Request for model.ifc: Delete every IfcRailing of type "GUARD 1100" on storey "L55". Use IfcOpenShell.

First a look at what the model holds.

```python
import ifcopenshell
import ifcopenshell.util.element

model = ifcopenshell.open("model.ifc")
print(model.schema)
storey = next(s for s in model.by_type("IfcBuildingStorey") if s.Name == "L55")
railings = [e for e in ifcopenshell.util.element.get_decomposition(storey) if e.is_a("IfcRailing")]
seen = {}
for e in railings:
    element_type = ifcopenshell.util.element.get_type(e)
    name = element_type.Name if element_type not in (None, e) else None
    seen[name] = seen.get(name, 0) + 1
for name, count in sorted(seen.items(), key=str):
    print(count, "x", name)
```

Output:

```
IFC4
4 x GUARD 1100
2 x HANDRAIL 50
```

```python
import ifcopenshell
import ifcopenshell.api.root
import ifcopenshell.util.element

model = ifcopenshell.open("model.ifc")

storey = next(s for s in model.by_type("IfcBuildingStorey") if s.Name == "L55")
railings = [e for e in ifcopenshell.util.element.get_decomposition(storey) if e.is_a("IfcRailing")]
targets = [e for e in railings if (t := ifcopenshell.util.element.get_type(e)) not in (None, e) and t.Name == "GUARD 1100"]

for e in targets:
    ifcopenshell.api.root.remove_product(model, product=e)
print(len(targets), "removed")

model.write("model_edited.ifc")
```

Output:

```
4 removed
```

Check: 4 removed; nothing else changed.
